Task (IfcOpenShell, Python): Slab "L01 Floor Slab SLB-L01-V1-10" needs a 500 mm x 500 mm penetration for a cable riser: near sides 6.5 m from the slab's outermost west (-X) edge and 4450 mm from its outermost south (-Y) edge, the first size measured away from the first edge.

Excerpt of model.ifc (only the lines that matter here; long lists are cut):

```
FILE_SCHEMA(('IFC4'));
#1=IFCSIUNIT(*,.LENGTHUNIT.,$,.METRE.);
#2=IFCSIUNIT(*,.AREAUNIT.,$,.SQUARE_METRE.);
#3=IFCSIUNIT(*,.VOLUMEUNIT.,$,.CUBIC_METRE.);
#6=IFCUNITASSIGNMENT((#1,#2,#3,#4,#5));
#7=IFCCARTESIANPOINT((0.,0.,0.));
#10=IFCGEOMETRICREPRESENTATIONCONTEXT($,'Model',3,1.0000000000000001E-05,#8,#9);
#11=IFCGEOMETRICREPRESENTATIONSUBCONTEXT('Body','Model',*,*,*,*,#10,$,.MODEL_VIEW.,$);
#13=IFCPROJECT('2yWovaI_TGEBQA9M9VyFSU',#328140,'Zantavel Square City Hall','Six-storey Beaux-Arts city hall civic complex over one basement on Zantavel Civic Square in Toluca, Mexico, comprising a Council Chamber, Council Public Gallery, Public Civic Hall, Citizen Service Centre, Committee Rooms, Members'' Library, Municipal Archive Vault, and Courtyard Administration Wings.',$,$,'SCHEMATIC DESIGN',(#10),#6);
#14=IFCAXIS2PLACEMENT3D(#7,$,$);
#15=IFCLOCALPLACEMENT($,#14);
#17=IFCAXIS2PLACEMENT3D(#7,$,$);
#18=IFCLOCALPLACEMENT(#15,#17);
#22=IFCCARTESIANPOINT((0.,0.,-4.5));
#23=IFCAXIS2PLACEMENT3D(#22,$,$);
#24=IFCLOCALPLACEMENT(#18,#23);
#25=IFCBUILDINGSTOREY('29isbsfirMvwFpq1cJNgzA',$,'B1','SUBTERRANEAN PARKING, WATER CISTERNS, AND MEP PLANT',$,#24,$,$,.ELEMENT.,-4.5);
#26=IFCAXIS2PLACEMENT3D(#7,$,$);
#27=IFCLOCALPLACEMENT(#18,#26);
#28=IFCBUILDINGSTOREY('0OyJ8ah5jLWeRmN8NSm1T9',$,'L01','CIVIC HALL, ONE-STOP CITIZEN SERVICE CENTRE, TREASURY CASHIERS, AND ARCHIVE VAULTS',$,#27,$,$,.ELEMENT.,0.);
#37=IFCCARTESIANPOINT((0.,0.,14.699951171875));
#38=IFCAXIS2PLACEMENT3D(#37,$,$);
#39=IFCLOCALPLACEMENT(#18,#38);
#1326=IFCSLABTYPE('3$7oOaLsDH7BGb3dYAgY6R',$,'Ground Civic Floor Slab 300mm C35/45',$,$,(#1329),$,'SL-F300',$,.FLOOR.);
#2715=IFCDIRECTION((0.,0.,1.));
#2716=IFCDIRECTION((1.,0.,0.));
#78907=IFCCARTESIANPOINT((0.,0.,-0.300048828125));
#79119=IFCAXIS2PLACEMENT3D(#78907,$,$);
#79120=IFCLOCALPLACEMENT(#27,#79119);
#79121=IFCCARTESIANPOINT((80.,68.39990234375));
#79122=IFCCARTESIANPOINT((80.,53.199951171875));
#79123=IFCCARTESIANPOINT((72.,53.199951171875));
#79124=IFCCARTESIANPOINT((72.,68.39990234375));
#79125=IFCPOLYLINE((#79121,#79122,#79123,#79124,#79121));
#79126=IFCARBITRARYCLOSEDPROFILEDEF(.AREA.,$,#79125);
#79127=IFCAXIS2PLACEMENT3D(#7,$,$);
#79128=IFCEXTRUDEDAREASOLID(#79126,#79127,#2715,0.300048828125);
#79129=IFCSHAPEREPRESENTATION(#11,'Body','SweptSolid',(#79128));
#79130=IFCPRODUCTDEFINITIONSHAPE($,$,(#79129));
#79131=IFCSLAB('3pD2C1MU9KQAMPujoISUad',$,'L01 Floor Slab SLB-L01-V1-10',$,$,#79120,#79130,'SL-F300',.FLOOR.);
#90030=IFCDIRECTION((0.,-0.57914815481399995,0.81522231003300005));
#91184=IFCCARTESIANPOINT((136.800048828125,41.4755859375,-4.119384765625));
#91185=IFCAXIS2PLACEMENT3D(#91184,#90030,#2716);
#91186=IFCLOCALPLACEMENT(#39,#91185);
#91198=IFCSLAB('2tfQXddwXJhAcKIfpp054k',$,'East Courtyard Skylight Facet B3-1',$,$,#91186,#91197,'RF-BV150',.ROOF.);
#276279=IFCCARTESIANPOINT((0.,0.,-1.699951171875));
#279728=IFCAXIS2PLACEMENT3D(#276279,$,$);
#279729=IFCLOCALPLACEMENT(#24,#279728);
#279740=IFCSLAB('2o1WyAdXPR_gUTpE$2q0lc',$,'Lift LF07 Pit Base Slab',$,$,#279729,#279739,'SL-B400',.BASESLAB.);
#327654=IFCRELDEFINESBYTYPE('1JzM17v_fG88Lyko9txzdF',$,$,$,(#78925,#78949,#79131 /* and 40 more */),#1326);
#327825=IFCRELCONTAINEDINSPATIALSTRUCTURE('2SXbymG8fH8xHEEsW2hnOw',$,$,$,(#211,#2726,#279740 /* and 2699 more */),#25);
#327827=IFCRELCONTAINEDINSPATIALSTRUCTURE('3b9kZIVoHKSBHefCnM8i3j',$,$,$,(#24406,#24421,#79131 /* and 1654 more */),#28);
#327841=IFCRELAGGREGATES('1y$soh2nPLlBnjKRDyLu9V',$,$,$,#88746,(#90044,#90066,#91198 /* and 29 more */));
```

```python
import numpy as np
import ifcopenshell
import ifcopenshell.api.feature
import ifcopenshell.api.geometry
import ifcopenshell.api.root
import ifcopenshell.geom
import ifcopenshell.util.placement
import ifcopenshell.util.representation
import ifcopenshell.util.shape
import ifcopenshell.util.unit

model = ifcopenshell.open("model.ifc")
unit_scale = ifcopenshell.util.unit.calculate_unit_scale(model)
settings = ifcopenshell.geom.settings()


def volume(element):
    """Net volume in cubic metres, openings subtracted."""
    shape = ifcopenshell.geom.create_shape(settings, element)
    return ifcopenshell.util.shape.get_volume(shape.geometry)


slab = model.by_guid("3pD2C1MU9KQAMPujoISUad")
before = volume(slab)

# Extent in the slab's own axes, in metres. The edges named are its -X and -Y sides.
slab_shape = ifcopenshell.geom.create_shape(settings, slab)
vertices = ifcopenshell.util.shape.get_vertices(slab_shape.geometry)
x_min, y_min, bottom = vertices.min(axis=0)
top = vertices[:, 2].max()

opening = ifcopenshell.api.root.create_entity(model, ifc_class="IfcOpeningElement", name="Cable riser opening", predefined_type="OPENING")
context = ifcopenshell.util.representation.get_context(model, "Model", "Body", "MODEL_VIEW")
width, depth = 0.5, 0.5
outline = [(0.0, 0.0), (width, 0.0), (width, depth), (0.0, depth), (0.0, 0.0)]
# Overshoot both faces by 50 mm so the cut is clean.
shape = ifcopenshell.api.geometry.add_slab_representation(
    model, context=context, depth=top - bottom + 0.1, polyline=outline
)
ifcopenshell.api.geometry.assign_representation(model, product=opening, representation=shape)

matrix = ifcopenshell.util.placement.get_local_placement(slab.ObjectPlacement)
matrix[:, 3] = matrix @ np.append(np.array([x_min + 6.5, y_min + 4.45, bottom - 0.05]) / unit_scale, 1.0)
ifcopenshell.api.geometry.edit_object_placement(model, product=opening, matrix=matrix, is_si=False)
ifcopenshell.api.feature.add_feature(model, feature=opening, element=slab)

after = volume(slab)

print(f"slab volume {before:.3f} -> {after:.3f} m3")

model.write("model-out.ifc")
```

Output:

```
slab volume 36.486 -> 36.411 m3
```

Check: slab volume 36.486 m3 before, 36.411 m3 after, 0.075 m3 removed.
